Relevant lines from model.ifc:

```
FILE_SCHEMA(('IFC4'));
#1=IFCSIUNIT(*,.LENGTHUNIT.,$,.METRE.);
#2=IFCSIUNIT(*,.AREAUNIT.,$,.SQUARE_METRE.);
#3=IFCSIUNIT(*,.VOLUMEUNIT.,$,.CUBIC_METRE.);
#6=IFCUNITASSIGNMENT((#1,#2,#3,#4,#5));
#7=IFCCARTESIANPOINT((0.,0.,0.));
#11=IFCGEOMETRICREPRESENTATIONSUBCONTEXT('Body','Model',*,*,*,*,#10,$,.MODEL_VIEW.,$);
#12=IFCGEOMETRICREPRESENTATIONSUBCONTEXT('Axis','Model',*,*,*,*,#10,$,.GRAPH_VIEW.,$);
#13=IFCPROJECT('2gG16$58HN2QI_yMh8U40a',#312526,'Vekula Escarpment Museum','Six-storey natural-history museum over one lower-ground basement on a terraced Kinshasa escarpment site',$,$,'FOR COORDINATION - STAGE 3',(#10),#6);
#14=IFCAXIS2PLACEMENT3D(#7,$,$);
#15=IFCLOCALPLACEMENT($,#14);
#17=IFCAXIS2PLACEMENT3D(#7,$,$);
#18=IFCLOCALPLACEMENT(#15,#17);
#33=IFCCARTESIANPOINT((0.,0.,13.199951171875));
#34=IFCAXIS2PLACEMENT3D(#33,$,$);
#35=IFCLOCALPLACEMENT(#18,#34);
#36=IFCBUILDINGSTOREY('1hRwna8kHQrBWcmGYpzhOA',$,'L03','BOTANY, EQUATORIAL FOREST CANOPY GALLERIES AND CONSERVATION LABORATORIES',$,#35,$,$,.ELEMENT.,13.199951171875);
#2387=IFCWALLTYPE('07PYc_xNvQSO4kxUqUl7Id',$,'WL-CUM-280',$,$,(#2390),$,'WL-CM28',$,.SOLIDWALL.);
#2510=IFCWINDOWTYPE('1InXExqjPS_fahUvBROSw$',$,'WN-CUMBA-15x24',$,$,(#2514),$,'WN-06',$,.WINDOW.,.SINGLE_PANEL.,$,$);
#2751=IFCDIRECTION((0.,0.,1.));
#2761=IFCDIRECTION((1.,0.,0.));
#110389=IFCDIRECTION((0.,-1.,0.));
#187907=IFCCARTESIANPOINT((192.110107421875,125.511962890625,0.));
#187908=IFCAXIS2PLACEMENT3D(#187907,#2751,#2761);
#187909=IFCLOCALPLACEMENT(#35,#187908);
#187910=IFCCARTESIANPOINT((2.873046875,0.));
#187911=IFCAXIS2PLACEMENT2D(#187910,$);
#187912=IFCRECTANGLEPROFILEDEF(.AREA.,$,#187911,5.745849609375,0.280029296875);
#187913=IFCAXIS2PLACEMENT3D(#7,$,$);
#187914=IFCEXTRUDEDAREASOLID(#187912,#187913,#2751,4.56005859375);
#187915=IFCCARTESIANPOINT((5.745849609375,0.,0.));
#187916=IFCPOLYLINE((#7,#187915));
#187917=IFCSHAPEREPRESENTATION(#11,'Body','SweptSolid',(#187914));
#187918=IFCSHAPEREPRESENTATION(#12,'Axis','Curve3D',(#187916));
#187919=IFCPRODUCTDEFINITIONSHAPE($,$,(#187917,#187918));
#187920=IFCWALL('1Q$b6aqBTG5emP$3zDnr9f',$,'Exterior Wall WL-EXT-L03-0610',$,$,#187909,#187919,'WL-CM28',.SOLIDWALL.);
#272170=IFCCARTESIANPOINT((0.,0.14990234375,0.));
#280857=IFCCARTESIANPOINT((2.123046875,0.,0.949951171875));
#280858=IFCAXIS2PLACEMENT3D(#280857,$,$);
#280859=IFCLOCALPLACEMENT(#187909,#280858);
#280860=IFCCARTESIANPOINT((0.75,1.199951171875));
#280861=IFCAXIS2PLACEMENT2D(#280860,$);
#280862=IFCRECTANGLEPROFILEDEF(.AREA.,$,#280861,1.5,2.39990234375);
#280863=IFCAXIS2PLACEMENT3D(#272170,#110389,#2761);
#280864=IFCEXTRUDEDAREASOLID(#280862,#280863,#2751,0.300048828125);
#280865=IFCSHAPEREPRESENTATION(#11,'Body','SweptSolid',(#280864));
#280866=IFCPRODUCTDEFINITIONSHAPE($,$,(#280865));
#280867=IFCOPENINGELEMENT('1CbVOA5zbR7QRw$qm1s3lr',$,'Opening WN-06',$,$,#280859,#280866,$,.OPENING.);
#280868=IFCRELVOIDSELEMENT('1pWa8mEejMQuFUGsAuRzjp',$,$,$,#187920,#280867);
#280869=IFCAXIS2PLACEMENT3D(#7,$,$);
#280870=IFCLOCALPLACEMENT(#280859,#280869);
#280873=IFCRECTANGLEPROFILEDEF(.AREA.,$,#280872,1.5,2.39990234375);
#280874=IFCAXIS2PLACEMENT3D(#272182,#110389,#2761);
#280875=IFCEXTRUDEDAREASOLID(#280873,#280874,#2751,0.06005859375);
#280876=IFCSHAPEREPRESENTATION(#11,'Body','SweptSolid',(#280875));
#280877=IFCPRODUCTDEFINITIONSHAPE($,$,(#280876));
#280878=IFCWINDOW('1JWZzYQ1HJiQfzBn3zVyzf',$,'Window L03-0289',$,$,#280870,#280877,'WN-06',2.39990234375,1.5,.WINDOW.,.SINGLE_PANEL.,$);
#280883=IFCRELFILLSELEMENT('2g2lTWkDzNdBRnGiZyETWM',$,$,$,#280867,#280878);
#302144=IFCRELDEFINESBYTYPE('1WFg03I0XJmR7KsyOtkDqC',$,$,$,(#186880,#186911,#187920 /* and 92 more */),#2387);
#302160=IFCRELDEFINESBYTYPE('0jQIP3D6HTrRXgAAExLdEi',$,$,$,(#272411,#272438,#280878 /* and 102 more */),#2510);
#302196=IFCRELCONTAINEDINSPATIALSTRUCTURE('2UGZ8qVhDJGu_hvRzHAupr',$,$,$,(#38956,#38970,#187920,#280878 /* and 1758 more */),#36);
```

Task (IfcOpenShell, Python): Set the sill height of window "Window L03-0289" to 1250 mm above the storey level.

```python
import numpy as np
import ifcopenshell
import ifcopenshell.api.geometry
import ifcopenshell.geom
import ifcopenshell.util.element
import ifcopenshell.util.placement
import ifcopenshell.util.shape
import ifcopenshell.util.unit

model = ifcopenshell.open("model.ifc")
unit_scale = ifcopenshell.util.unit.calculate_unit_scale(model)

window = model.by_guid("1JWZzYQ1HJiQfzBn3zVyzf")
opening = window.FillsVoids[0].RelatingOpeningElement
storey = ifcopenshell.util.element.get_container(window, ifc_class="IfcBuildingStorey")
level = ifcopenshell.util.placement.get_local_placement(storey.ObjectPlacement)[2, 3]

# The opening's origin need not be at the sill, so measure its lowest point.
shape = ifcopenshell.geom.create_shape(ifcopenshell.geom.settings(), opening)
bottom = ifcopenshell.util.shape.get_shape_bottom_elevation(shape, shape.geometry) / unit_scale
dz = level + 1.25 / unit_scale - bottom

shift = np.array([0.0, 0.0, dz])
# The window is placed relative to its opening, so it follows when the opening moves.
matrix = ifcopenshell.util.placement.get_local_placement(opening.ObjectPlacement)
matrix[:3, 3] += shift
ifcopenshell.api.geometry.edit_object_placement(
    model, product=opening, matrix=matrix, is_si=False, should_transform_children=True
)

print(f"moved by {dz * unit_scale:+.3f} m")

model.write("model_edited.ifc")
```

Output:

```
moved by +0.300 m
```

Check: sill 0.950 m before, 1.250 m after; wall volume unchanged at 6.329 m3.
